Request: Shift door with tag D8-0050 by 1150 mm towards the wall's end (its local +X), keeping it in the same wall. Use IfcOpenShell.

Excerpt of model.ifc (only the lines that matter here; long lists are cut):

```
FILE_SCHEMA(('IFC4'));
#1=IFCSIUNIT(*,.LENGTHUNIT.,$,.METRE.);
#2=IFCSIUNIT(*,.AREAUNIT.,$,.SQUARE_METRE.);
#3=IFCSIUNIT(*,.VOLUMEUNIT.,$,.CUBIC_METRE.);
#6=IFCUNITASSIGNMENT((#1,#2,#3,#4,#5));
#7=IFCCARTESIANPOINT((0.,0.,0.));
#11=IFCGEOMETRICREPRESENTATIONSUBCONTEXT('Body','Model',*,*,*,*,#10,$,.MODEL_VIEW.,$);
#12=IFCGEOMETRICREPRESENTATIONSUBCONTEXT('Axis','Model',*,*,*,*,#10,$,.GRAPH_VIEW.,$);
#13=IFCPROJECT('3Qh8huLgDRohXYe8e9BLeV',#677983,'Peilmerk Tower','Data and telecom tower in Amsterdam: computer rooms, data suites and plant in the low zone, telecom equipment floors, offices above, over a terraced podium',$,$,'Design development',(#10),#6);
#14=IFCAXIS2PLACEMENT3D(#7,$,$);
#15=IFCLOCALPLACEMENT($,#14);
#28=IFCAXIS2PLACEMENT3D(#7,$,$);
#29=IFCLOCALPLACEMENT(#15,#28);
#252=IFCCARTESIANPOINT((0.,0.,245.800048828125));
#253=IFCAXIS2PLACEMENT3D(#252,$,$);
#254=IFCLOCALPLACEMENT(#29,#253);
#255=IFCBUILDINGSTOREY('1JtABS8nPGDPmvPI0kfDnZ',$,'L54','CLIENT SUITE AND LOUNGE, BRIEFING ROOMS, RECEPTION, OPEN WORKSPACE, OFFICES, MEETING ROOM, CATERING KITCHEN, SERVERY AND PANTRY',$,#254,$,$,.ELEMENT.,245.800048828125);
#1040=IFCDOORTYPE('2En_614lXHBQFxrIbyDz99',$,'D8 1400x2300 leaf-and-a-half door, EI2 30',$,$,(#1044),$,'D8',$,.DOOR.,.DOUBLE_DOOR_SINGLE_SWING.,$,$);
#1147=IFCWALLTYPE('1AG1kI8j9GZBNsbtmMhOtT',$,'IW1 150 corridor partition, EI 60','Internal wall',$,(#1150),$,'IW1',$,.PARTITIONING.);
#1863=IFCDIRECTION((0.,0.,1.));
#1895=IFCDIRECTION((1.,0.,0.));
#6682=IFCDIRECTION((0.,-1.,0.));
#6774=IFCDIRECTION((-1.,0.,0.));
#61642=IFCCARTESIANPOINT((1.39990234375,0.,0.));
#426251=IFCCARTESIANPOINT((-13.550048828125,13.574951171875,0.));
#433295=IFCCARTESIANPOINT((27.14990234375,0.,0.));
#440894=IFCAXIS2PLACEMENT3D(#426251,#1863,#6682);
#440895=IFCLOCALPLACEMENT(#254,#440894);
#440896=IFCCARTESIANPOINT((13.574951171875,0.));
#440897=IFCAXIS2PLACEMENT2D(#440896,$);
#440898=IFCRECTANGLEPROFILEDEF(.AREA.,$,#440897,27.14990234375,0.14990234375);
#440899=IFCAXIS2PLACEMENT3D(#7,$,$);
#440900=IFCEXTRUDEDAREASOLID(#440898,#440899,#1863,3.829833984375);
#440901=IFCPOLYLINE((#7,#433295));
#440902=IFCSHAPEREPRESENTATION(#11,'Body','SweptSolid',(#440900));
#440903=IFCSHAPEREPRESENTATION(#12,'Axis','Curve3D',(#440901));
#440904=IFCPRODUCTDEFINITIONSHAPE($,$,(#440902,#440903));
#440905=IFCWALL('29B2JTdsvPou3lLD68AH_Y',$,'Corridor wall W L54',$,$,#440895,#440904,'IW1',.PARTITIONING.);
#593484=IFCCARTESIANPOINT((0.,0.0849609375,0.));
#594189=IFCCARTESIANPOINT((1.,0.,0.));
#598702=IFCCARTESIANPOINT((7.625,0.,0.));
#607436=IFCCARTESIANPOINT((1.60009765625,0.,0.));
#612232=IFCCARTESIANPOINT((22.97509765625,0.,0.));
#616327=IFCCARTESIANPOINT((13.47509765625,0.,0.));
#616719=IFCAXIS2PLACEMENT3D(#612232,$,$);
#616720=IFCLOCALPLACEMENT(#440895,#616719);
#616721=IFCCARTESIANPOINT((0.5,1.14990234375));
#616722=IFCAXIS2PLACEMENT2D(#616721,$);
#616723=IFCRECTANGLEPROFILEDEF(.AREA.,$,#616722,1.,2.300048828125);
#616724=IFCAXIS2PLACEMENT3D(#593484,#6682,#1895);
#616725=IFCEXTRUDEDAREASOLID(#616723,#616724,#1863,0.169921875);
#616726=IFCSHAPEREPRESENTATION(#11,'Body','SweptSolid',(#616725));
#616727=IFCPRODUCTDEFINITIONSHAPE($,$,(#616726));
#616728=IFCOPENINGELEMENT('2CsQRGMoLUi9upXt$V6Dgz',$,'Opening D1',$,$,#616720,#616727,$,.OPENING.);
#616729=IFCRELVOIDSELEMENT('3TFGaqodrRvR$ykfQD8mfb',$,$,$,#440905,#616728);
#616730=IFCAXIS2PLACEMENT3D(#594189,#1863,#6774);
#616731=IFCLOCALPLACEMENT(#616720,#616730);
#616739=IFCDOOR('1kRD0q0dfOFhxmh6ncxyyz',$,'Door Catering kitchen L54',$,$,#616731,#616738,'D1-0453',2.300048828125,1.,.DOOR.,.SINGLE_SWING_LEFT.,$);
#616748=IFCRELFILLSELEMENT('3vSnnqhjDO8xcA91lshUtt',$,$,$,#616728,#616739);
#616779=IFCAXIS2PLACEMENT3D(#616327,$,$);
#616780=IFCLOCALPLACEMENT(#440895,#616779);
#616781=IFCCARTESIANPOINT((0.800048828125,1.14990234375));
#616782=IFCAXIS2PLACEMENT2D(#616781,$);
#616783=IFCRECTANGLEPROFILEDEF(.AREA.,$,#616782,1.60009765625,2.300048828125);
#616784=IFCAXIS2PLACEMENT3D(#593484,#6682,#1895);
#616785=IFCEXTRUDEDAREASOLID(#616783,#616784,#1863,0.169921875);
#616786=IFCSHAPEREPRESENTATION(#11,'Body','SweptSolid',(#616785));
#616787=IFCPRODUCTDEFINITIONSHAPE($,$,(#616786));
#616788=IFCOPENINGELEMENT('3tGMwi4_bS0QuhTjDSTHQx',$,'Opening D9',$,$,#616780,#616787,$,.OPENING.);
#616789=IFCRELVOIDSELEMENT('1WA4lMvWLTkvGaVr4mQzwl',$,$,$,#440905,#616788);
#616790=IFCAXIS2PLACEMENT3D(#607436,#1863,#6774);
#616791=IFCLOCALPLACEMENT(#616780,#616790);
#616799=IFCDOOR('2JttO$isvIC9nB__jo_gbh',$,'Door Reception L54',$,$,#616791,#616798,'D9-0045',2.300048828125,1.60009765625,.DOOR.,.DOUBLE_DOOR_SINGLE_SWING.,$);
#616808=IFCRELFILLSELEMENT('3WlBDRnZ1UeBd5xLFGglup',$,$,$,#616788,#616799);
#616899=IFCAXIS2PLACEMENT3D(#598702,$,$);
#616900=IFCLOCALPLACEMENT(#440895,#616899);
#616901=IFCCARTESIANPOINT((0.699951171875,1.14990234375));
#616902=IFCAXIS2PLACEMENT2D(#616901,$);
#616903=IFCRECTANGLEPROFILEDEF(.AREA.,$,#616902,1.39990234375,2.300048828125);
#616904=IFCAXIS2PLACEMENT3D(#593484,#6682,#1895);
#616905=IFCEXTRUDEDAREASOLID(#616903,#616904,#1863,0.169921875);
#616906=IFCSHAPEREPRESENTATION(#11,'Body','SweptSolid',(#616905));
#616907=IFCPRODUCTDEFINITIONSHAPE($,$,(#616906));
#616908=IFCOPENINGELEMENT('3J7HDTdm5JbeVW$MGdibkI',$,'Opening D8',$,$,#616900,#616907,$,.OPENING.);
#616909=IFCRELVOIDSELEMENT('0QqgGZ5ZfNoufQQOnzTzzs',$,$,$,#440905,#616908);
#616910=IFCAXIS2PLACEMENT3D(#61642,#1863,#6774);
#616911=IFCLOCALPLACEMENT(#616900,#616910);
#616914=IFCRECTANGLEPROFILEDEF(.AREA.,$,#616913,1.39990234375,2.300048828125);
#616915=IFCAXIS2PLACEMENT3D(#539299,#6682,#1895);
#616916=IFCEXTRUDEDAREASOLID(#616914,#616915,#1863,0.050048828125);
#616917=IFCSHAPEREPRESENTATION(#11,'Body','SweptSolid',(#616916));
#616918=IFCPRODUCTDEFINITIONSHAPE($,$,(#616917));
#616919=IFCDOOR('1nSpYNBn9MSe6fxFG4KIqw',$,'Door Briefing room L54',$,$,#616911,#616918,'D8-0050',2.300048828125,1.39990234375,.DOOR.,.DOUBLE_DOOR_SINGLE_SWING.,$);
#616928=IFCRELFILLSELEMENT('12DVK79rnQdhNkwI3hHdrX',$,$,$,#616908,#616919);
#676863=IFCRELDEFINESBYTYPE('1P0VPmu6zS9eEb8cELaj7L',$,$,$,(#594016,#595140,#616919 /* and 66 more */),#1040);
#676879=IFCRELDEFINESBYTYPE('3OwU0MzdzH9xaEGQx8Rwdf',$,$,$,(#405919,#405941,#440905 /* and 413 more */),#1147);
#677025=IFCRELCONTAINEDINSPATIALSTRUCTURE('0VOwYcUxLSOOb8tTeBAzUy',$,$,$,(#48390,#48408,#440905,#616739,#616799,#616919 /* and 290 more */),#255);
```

```python
import ifcopenshell
import ifcopenshell.api.geometry
import ifcopenshell.util.placement

model = ifcopenshell.open("model.ifc")

door = model.by_guid("1nSpYNBn9MSe6fxFG4KIqw")
opening = door.FillsVoids[0].RelatingOpeningElement
wall = opening.VoidsElements[0].RelatingBuildingElement

wall_matrix = ifcopenshell.util.placement.get_local_placement(wall.ObjectPlacement)
shift = wall_matrix[:3, 0] * 1.15
before = ifcopenshell.util.placement.get_local_placement(door.ObjectPlacement)[:3, 3].copy()

# The door is placed relative to its opening, so it follows when the opening moves.
matrix = ifcopenshell.util.placement.get_local_placement(opening.ObjectPlacement)
matrix[:3, 3] += shift
ifcopenshell.api.geometry.edit_object_placement(
    model, product=opening, matrix=matrix, is_si=False, should_transform_children=True
)

after = ifcopenshell.util.placement.get_local_placement(door.ObjectPlacement)[:3, 3]
print("door moved by", (after - before).round(3) + 0.0)

model.write("model-out.ifc")
```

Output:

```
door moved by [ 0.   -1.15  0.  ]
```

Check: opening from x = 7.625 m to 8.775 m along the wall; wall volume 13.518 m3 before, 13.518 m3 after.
